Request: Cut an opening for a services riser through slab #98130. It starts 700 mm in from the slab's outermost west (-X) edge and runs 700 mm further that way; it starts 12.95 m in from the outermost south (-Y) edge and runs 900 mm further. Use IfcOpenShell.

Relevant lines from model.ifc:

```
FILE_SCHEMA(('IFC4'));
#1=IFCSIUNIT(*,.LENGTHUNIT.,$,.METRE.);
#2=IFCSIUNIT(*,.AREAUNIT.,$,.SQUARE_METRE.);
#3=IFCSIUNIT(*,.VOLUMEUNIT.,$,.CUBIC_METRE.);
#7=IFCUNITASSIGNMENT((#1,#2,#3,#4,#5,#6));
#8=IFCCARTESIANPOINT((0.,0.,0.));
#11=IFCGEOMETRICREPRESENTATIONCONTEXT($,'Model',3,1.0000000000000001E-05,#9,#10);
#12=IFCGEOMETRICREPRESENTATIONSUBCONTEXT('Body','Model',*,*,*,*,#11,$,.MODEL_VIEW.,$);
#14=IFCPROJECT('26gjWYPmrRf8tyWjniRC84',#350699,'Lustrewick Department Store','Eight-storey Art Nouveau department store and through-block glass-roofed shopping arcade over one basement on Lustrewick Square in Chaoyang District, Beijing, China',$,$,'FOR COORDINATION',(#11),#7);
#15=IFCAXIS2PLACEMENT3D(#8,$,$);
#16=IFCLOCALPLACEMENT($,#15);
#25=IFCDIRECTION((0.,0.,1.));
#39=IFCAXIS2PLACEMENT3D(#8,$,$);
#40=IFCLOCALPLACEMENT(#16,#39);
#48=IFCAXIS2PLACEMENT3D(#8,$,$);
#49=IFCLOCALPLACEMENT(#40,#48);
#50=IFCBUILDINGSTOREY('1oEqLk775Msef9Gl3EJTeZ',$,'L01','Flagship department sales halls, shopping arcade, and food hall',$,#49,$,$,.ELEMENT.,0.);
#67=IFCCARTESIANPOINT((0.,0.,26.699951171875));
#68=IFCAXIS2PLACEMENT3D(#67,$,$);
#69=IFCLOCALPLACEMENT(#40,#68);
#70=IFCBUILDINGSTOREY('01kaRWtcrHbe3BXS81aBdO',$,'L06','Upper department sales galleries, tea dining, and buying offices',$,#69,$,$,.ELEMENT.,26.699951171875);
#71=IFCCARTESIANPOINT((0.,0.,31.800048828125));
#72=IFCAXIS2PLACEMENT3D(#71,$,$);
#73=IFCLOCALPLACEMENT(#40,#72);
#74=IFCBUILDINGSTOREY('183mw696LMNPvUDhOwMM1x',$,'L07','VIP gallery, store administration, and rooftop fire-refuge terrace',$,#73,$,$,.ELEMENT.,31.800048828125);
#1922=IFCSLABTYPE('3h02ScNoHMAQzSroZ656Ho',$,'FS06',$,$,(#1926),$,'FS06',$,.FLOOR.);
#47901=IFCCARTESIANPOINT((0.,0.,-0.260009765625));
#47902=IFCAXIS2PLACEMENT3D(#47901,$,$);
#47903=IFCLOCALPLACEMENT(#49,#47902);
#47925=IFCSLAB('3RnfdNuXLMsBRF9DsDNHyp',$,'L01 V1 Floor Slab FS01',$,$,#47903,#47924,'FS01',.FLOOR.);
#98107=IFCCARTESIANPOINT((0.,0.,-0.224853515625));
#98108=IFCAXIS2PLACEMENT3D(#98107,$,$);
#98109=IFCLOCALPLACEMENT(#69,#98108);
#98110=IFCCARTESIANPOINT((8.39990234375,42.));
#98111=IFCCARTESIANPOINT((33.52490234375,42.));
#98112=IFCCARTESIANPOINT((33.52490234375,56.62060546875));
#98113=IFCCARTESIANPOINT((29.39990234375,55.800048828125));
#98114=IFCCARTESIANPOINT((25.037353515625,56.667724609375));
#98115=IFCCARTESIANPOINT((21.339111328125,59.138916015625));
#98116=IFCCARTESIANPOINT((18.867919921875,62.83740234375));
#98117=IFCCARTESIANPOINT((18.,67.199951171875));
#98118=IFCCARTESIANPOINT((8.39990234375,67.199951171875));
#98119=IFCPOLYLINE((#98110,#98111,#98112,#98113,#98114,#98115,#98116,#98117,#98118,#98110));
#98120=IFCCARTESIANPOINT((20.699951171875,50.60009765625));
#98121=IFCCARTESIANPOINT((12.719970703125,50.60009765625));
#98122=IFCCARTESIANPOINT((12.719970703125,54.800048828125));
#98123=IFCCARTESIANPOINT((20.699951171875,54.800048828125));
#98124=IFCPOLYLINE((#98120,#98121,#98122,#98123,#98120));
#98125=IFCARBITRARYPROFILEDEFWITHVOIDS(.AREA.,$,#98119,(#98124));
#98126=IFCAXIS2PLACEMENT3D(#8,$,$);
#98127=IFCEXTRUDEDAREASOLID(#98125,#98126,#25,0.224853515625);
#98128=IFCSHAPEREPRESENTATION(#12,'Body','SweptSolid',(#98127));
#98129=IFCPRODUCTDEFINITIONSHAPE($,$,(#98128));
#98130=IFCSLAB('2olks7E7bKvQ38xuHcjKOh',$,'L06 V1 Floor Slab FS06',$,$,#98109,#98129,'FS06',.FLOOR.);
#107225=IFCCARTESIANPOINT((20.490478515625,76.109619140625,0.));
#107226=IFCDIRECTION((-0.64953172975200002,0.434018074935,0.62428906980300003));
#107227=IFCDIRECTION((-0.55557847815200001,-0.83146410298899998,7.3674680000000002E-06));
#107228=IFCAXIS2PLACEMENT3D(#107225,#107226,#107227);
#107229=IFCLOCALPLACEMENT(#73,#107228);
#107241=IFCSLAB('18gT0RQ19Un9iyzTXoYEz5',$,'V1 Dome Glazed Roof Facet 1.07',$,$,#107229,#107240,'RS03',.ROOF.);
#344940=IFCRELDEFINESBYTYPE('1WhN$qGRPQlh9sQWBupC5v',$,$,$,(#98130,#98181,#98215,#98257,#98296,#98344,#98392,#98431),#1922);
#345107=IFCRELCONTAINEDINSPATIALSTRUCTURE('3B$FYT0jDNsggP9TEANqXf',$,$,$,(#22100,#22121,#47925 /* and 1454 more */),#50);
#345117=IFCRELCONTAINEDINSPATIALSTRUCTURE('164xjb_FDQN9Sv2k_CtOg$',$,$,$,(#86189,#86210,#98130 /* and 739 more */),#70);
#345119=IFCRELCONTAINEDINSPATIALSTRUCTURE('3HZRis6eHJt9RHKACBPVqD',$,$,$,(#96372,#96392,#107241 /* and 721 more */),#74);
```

```python
import numpy as np
import ifcopenshell
import ifcopenshell.api.feature
import ifcopenshell.api.geometry
import ifcopenshell.api.root
import ifcopenshell.geom
import ifcopenshell.util.placement
import ifcopenshell.util.representation
import ifcopenshell.util.shape
import ifcopenshell.util.unit

model = ifcopenshell.open("model.ifc")
unit_scale = ifcopenshell.util.unit.calculate_unit_scale(model)
settings = ifcopenshell.geom.settings()


def volume(element):
    """Net volume in cubic metres, openings subtracted."""
    shape = ifcopenshell.geom.create_shape(settings, element)
    return ifcopenshell.util.shape.get_volume(shape.geometry)


slab = model.by_guid("2olks7E7bKvQ38xuHcjKOh")
before = volume(slab)

# Extent in the slab's own axes, in metres. The edges named are its -X and -Y sides.
slab_shape = ifcopenshell.geom.create_shape(settings, slab)
vertices = ifcopenshell.util.shape.get_vertices(slab_shape.geometry)
x_min, y_min, bottom = vertices.min(axis=0)
top = vertices[:, 2].max()

opening = ifcopenshell.api.root.create_entity(model, ifc_class="IfcOpeningElement", name="Services riser opening", predefined_type="OPENING")
context = ifcopenshell.util.representation.get_context(model, "Model", "Body", "MODEL_VIEW")
width, depth = 0.7, 0.9
outline = [(0.0, 0.0), (width, 0.0), (width, depth), (0.0, depth), (0.0, 0.0)]
# Overshoot both faces by 50 mm so the cut is clean.
shape = ifcopenshell.api.geometry.add_slab_representation(
    model, context=context, depth=top - bottom + 0.1, polyline=outline
)
ifcopenshell.api.geometry.assign_representation(model, product=opening, representation=shape)

matrix = ifcopenshell.util.placement.get_local_placement(slab.ObjectPlacement)
matrix[:, 3] = matrix @ np.append(np.array([x_min + 0.7, y_min + 12.95, bottom - 0.05]) / unit_scale, 1.0)
ifcopenshell.api.geometry.edit_object_placement(model, product=opening, matrix=matrix, is_si=False)
ifcopenshell.api.feature.add_feature(model, feature=opening, element=slab)

after = volume(slab)

print(f"slab volume {before:.3f} -> {after:.3f} m3")

model.write("model-out.ifc")
```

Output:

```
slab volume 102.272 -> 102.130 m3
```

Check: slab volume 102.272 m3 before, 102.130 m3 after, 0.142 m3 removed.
